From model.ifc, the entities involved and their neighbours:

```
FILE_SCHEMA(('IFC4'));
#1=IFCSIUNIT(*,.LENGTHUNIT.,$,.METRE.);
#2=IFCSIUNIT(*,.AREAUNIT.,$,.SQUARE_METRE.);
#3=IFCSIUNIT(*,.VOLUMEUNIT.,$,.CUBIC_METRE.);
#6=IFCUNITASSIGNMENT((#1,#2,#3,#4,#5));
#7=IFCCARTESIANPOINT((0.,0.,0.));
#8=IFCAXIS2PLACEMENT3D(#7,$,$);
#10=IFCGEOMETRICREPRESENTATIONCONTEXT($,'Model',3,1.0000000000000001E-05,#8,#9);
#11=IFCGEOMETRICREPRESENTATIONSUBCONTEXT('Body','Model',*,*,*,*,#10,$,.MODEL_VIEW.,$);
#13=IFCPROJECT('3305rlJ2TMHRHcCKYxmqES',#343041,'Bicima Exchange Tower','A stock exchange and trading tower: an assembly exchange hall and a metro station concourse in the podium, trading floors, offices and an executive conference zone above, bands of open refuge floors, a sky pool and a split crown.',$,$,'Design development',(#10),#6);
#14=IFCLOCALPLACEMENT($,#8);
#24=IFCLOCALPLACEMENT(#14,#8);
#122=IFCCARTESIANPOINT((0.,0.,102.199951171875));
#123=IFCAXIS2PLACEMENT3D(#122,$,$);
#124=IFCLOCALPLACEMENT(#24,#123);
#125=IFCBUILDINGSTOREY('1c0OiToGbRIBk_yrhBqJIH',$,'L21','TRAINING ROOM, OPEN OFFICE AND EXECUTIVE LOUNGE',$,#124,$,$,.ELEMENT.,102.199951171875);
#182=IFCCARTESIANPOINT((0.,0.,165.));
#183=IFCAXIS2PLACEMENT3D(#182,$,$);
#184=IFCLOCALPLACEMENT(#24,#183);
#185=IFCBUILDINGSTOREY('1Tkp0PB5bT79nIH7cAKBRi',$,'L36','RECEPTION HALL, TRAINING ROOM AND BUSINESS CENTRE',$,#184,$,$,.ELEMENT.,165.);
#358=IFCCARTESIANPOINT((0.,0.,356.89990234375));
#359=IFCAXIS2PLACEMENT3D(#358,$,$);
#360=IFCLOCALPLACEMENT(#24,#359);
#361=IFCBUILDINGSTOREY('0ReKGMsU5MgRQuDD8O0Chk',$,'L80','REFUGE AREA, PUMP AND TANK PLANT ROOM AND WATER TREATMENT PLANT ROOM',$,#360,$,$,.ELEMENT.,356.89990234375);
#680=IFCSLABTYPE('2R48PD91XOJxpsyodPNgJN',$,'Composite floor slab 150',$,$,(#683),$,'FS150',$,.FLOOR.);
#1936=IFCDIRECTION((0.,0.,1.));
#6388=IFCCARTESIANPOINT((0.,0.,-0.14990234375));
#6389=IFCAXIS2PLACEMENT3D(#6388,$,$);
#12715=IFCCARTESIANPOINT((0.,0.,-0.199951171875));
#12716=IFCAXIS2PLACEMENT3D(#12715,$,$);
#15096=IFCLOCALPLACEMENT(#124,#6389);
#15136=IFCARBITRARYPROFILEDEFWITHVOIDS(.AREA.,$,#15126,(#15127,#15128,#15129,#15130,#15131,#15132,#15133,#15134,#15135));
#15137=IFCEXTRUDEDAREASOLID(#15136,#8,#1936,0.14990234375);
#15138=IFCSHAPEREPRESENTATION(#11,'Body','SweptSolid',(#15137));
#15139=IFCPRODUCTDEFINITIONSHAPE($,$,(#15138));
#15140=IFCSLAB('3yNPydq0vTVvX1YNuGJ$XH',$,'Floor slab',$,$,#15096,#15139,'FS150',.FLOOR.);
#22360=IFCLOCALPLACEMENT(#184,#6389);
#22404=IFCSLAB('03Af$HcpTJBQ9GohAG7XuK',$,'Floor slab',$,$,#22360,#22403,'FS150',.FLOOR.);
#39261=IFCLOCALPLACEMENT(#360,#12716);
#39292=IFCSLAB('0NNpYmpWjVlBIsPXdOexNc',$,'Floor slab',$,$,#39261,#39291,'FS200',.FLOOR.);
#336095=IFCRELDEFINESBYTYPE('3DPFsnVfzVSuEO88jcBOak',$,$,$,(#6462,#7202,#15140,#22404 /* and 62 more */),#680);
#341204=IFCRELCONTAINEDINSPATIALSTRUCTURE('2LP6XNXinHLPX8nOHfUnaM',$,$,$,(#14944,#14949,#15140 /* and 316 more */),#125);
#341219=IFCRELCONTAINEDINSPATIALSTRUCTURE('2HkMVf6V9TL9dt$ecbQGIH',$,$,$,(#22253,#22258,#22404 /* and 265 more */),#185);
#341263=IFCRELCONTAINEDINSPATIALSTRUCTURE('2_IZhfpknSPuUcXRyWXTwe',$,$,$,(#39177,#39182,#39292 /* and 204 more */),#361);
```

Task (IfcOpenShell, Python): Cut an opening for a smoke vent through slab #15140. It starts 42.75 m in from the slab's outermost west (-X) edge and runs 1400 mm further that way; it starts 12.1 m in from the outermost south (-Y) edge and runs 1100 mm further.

```python
import numpy as np
import ifcopenshell
import ifcopenshell.api.feature
import ifcopenshell.api.geometry
import ifcopenshell.api.root
import ifcopenshell.geom
import ifcopenshell.util.placement
import ifcopenshell.util.representation
import ifcopenshell.util.shape
import ifcopenshell.util.unit

model = ifcopenshell.open("model.ifc")
unit_scale = ifcopenshell.util.unit.calculate_unit_scale(model)
settings = ifcopenshell.geom.settings()


def volume(element):
    """Net volume in cubic metres, openings subtracted."""
    shape = ifcopenshell.geom.create_shape(settings, element)
    return ifcopenshell.util.shape.get_volume(shape.geometry)


slab = model.by_guid("3yNPydq0vTVvX1YNuGJ$XH")
before = volume(slab)

# Extent in the slab's own axes, in metres. The edges named are its -X and -Y sides.
slab_shape = ifcopenshell.geom.create_shape(settings, slab)
vertices = ifcopenshell.util.shape.get_vertices(slab_shape.geometry)
x_min, y_min, bottom = vertices.min(axis=0)
top = vertices[:, 2].max()

opening = ifcopenshell.api.root.create_entity(model, ifc_class="IfcOpeningElement", name="Smoke vent opening", predefined_type="OPENING")
context = ifcopenshell.util.representation.get_context(model, "Model", "Body", "MODEL_VIEW")
width, depth = 1.4, 1.1
outline = [(0.0, 0.0), (width, 0.0), (width, depth), (0.0, depth), (0.0, 0.0)]
# Overshoot both faces by 50 mm so the cut is clean.
shape = ifcopenshell.api.geometry.add_slab_representation(
    model, context=context, depth=top - bottom + 0.1, polyline=outline
)
ifcopenshell.api.geometry.assign_representation(model, product=opening, representation=shape)

matrix = ifcopenshell.util.placement.get_local_placement(slab.ObjectPlacement)
matrix[:, 3] = matrix @ np.append(np.array([x_min + 42.75, y_min + 12.1, bottom - 0.05]) / unit_scale, 1.0)
ifcopenshell.api.geometry.edit_object_placement(model, product=opening, matrix=matrix, is_si=False)
ifcopenshell.api.feature.add_feature(model, feature=opening, element=slab)

after = volume(slab)

print(f"slab volume {before:.3f} -> {after:.3f} m3")

model.write("model-out.ifc")
```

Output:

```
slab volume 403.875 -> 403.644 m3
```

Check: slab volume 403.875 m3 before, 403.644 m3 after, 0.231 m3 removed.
